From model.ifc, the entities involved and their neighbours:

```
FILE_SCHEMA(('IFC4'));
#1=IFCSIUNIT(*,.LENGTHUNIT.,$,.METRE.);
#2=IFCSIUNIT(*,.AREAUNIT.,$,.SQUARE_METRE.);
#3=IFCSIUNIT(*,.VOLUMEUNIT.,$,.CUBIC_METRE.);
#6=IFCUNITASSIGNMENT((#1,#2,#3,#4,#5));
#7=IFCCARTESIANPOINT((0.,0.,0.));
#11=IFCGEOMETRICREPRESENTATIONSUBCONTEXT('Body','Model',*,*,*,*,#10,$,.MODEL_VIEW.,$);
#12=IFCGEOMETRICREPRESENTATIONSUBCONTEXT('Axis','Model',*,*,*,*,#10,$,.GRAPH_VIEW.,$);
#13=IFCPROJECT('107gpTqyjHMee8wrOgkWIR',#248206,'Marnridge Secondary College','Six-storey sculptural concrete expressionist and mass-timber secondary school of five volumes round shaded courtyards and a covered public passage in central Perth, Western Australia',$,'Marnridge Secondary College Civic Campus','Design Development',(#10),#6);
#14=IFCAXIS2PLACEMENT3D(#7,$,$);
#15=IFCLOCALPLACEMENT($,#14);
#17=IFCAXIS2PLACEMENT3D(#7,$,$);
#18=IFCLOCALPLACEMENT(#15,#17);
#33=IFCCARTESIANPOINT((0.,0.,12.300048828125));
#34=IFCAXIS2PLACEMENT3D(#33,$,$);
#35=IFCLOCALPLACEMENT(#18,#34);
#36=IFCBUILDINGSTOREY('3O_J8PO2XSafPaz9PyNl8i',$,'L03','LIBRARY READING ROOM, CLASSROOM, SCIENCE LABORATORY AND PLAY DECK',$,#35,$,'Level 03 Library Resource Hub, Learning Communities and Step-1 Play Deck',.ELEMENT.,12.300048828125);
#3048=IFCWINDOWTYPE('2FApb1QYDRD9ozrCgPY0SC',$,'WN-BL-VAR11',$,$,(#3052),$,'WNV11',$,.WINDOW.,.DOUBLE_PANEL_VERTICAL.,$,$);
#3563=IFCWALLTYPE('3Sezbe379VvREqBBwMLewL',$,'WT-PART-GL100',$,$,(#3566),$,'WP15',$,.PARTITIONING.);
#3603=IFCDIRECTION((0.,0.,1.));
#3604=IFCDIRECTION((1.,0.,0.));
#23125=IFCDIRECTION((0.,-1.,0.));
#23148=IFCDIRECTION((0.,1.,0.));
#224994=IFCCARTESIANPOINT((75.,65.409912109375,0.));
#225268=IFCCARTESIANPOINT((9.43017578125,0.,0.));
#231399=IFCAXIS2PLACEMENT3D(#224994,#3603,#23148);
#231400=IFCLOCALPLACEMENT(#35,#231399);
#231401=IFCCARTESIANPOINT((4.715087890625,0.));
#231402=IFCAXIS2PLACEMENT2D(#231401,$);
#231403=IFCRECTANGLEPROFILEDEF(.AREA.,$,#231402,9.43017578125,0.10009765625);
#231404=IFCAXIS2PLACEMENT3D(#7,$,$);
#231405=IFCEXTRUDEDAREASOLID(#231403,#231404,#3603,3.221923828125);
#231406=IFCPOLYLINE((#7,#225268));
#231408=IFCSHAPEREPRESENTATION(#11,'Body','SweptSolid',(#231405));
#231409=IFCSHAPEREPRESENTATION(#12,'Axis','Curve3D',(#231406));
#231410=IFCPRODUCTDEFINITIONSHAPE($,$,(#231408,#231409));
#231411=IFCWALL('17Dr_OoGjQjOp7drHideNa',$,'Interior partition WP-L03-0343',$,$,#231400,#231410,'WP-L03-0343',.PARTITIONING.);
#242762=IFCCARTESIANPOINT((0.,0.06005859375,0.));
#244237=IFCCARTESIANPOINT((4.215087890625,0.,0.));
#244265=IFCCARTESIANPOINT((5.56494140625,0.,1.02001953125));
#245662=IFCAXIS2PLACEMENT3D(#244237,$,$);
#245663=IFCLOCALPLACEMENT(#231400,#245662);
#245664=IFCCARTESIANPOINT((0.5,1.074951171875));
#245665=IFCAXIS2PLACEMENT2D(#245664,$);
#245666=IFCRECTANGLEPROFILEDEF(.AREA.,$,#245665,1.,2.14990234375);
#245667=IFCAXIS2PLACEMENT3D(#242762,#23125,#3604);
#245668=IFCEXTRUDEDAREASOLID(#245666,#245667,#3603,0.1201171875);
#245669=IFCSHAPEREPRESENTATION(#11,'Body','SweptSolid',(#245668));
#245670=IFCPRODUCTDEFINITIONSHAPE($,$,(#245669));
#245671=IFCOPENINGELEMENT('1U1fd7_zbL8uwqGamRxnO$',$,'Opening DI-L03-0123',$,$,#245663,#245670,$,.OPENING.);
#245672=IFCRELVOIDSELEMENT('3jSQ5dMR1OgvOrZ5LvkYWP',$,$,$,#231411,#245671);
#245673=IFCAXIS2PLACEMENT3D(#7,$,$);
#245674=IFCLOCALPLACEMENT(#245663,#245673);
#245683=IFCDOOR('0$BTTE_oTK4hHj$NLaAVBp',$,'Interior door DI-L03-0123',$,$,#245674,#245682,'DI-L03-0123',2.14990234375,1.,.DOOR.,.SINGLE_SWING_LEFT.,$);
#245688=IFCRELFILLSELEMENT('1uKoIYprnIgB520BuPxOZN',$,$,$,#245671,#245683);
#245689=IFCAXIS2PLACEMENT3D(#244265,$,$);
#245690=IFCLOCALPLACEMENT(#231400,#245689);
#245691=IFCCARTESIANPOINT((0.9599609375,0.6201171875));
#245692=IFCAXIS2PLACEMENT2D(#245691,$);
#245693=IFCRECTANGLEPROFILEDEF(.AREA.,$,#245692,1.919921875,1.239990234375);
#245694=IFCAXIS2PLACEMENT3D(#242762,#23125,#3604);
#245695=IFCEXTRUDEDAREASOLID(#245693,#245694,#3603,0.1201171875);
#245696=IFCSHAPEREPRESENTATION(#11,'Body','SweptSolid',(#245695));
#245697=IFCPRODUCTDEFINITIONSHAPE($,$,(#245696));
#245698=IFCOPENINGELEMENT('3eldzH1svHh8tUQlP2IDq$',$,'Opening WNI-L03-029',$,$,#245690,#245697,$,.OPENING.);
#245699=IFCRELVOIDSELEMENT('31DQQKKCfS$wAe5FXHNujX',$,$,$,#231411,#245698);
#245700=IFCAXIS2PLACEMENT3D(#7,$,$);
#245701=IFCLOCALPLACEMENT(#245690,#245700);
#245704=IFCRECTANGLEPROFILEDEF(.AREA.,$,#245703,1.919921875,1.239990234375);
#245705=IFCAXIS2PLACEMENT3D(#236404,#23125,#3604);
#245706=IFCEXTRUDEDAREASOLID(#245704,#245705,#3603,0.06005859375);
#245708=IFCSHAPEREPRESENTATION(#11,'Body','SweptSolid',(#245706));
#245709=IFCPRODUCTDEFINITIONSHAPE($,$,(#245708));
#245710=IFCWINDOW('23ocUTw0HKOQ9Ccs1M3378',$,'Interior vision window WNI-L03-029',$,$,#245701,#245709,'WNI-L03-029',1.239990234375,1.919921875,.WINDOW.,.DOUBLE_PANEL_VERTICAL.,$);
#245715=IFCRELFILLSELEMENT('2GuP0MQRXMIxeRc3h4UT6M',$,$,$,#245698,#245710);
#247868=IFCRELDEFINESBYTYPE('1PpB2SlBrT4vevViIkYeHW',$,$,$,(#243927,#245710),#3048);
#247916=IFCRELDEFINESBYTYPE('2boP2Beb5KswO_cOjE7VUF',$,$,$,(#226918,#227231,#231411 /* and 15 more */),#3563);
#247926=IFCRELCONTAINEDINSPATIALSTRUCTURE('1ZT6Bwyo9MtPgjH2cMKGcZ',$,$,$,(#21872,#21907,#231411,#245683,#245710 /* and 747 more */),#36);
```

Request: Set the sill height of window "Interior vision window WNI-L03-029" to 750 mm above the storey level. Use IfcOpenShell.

```python
import numpy as np
import ifcopenshell
import ifcopenshell.api.geometry
import ifcopenshell.geom
import ifcopenshell.util.element
import ifcopenshell.util.placement
import ifcopenshell.util.shape
import ifcopenshell.util.unit

model = ifcopenshell.open("model.ifc")
unit_scale = ifcopenshell.util.unit.calculate_unit_scale(model)

window = model.by_guid("23ocUTw0HKOQ9Ccs1M3378")
opening = window.FillsVoids[0].RelatingOpeningElement
storey = ifcopenshell.util.element.get_container(window, ifc_class="IfcBuildingStorey")
level = ifcopenshell.util.placement.get_local_placement(storey.ObjectPlacement)[2, 3]

# The opening's origin need not be at the sill, so measure its lowest point.
shape = ifcopenshell.geom.create_shape(ifcopenshell.geom.settings(), opening)
bottom = ifcopenshell.util.shape.get_shape_bottom_elevation(shape, shape.geometry) / unit_scale
dz = level + 0.75 / unit_scale - bottom

shift = np.array([0.0, 0.0, dz])
# The window is placed relative to its opening, so it follows when the opening moves.
matrix = ifcopenshell.util.placement.get_local_placement(opening.ObjectPlacement)
matrix[:3, 3] += shift
ifcopenshell.api.geometry.edit_object_placement(
    model, product=opening, matrix=matrix, is_si=False, should_transform_children=True
)

print(f"moved by {dz * unit_scale:+.3f} m")

model.write("model-out.ifc")
```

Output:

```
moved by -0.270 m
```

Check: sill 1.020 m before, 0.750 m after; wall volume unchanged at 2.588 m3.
